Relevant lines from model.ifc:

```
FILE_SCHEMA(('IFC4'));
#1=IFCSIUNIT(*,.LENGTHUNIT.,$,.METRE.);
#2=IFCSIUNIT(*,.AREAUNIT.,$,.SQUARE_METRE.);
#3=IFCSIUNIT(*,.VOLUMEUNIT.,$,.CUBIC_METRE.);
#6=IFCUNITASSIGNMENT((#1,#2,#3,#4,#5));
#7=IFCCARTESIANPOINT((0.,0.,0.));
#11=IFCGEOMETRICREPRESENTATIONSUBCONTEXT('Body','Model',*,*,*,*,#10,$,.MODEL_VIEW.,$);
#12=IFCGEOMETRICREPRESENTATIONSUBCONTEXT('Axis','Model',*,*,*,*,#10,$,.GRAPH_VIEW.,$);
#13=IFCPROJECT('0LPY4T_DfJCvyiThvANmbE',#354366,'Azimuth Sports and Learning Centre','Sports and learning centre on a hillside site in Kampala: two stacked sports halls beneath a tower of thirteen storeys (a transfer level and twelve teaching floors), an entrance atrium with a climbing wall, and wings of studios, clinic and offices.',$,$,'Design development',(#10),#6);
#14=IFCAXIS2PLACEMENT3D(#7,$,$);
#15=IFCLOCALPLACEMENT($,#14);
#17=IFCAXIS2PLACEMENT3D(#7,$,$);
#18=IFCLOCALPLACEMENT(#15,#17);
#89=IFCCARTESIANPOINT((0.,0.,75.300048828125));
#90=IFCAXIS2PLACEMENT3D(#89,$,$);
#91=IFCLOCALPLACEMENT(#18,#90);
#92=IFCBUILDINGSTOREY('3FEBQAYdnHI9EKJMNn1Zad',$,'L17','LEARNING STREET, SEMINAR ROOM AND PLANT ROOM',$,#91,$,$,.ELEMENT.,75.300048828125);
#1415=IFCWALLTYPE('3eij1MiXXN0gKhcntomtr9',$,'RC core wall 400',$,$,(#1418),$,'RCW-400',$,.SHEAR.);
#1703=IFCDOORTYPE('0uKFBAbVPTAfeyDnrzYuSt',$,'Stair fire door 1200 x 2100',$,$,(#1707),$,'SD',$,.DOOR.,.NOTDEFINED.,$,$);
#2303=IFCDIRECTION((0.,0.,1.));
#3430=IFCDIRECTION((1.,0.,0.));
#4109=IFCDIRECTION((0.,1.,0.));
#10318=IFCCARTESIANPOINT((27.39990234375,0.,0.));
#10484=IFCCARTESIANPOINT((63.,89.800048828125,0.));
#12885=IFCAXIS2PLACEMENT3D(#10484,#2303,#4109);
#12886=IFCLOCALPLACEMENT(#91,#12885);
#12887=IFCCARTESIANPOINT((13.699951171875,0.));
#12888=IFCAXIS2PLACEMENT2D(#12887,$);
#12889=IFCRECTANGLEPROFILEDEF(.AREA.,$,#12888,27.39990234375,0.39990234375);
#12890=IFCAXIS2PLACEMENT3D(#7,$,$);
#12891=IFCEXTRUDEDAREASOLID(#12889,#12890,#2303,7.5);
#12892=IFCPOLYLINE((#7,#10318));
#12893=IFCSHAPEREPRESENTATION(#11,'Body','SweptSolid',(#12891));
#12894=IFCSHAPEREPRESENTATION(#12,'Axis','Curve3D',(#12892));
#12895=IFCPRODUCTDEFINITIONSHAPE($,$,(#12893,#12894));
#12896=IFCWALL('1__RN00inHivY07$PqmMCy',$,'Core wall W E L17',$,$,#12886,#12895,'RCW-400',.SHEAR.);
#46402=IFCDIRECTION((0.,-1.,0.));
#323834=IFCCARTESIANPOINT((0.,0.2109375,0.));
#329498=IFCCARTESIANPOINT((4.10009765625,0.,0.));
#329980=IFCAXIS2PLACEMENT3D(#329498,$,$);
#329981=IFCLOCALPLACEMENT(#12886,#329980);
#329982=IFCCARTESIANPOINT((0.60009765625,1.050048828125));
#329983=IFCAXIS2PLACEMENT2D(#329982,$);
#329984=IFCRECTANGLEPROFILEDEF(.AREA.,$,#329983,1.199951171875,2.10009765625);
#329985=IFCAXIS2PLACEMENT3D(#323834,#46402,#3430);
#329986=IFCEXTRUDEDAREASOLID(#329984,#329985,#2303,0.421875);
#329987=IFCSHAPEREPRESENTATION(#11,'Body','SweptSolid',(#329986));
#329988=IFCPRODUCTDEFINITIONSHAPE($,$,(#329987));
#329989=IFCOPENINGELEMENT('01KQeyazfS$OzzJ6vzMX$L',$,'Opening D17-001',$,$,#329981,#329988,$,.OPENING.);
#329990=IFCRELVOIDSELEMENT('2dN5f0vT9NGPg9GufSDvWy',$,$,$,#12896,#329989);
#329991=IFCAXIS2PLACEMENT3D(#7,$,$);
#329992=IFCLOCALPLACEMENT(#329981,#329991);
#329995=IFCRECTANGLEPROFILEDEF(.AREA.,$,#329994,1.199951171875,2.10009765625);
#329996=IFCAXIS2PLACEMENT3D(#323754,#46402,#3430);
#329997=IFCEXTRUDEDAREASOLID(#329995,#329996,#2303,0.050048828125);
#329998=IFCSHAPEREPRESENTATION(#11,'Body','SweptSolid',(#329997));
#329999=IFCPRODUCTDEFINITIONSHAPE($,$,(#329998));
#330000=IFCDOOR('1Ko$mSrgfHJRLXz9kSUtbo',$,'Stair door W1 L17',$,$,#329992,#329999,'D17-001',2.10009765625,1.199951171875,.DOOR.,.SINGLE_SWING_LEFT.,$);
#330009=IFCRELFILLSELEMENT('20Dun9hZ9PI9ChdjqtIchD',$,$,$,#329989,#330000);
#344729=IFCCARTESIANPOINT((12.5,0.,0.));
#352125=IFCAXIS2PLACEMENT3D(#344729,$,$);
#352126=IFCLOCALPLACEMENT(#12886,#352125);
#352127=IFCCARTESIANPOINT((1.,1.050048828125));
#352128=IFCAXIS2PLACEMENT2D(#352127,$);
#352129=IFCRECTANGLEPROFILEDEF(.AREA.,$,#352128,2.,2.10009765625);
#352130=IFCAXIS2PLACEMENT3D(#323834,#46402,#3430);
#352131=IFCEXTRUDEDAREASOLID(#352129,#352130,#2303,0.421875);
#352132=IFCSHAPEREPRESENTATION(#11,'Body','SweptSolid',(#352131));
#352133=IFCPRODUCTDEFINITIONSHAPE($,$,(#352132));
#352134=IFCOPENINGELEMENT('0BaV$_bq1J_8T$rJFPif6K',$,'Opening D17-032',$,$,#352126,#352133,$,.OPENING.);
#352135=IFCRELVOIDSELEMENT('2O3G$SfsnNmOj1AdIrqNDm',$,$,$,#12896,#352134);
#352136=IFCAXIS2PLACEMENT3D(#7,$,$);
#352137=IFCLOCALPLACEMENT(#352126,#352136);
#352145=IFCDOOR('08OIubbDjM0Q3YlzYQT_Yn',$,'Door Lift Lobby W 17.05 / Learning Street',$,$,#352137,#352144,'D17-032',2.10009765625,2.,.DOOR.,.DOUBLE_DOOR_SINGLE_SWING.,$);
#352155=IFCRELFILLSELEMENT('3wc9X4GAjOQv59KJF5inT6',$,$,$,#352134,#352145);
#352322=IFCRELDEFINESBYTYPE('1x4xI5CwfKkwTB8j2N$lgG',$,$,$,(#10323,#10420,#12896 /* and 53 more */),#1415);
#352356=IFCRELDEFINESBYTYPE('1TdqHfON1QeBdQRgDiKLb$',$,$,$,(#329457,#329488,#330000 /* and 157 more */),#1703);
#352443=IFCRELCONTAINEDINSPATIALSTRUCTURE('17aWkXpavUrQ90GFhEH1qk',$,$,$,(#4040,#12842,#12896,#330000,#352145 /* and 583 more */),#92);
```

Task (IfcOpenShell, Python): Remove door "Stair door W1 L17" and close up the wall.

```python
import ifcopenshell
import ifcopenshell.api.feature
import ifcopenshell.api.root
import ifcopenshell.geom
import ifcopenshell.util.shape

model = ifcopenshell.open("model.ifc")
settings = ifcopenshell.geom.settings()


def volume(element):
    """Net volume in cubic metres, openings subtracted."""
    shape = ifcopenshell.geom.create_shape(settings, element)
    return ifcopenshell.util.shape.get_volume(shape.geometry)


door = model.by_guid("1Ko$mSrgfHJRLXz9kSUtbo")
opening = door.FillsVoids[0].RelatingOpeningElement
wall = opening.VoidsElements[0].RelatingBuildingElement
before = volume(wall)

ifcopenshell.api.root.remove_product(model, product=door)
ifcopenshell.api.feature.remove_feature(model, feature=opening)

after = volume(wall)

print(f"wall volume {before:.3f} -> {after:.3f} m3")

model.write("model-out.ifc")
```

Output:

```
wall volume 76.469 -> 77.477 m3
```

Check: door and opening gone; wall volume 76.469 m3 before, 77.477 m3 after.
